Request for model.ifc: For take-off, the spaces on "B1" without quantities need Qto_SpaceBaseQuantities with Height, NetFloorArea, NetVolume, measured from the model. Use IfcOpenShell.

First a look at what the model holds.

```python
import ifcopenshell
import ifcopenshell.util.element
import ifcopenshell.util.unit

model = ifcopenshell.open("model.ifc")
print(model.schema)
for unit_type in ("LENGTHUNIT", "AREAUNIT", "VOLUMEUNIT"):
    print(unit_type, ifcopenshell.util.unit.calculate_unit_scale(model, unit_type))
storey = next(s for s in model.by_type("IfcBuildingStorey") if s.Name == "B1")
spaces = [e for e in ifcopenshell.util.element.get_decomposition(storey) if e.is_a("IfcSpace")]
for e in sorted(spaces, key=lambda e: e.id()):
    print(e.id(), e.is_a(), e.Name, list(ifcopenshell.util.element.get_psets(e, qtos_only=True)), sep=" | ")
```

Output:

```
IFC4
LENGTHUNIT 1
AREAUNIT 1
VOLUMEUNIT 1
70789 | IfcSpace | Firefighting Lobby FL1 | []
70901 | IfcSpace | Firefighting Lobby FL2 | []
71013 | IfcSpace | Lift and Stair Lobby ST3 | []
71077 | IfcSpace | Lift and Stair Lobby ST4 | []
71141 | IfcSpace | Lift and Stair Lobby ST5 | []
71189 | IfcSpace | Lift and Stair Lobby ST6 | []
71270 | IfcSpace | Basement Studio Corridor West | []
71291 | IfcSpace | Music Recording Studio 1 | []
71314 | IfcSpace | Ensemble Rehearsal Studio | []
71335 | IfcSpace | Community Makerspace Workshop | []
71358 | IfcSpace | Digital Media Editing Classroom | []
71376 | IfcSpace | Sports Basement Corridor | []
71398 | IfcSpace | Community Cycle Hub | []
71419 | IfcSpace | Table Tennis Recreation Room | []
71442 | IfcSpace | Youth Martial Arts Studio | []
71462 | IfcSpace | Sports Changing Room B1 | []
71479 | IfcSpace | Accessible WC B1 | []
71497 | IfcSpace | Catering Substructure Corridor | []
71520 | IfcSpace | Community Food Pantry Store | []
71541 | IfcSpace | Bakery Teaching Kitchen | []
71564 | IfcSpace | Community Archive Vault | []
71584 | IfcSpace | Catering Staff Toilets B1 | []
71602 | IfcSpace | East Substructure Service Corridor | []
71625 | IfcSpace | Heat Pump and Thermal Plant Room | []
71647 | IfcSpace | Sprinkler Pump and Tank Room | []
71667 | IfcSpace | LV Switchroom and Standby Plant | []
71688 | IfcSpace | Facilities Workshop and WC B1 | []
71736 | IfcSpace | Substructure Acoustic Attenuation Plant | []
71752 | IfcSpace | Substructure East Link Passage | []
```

```python
import ifcopenshell
import ifcopenshell.api.pset
import ifcopenshell.geom
import ifcopenshell.util.element
import ifcopenshell.util.shape
import ifcopenshell.util.unit

model = ifcopenshell.open("model.ifc")
unit_scale = ifcopenshell.util.unit.calculate_unit_scale(model)
area_scale = ifcopenshell.util.unit.calculate_unit_scale(model, "AREAUNIT")
volume_scale = ifcopenshell.util.unit.calculate_unit_scale(model, "VOLUMEUNIT")
settings = ifcopenshell.geom.settings()

storey = next(s for s in model.by_type("IfcBuildingStorey") if s.Name == "B1")
spaces = [e for e in ifcopenshell.util.element.get_decomposition(storey) if e.is_a("IfcSpace")]

for e in sorted(spaces, key=lambda e: e.id()):
    if ifcopenshell.util.element.get_psets(e, qtos_only=True, should_inherit=False):
        continue
    # Geometry comes back in metres, in the element's own axes.
    shape = ifcopenshell.geom.create_shape(settings, e)
    values = {
        "Height": ifcopenshell.util.shape.get_z(shape.geometry) / unit_scale,
        "NetFloorArea": ifcopenshell.util.shape.get_footprint_area(shape.geometry) / area_scale,
        "NetVolume": ifcopenshell.util.shape.get_volume(shape.geometry) / volume_scale,
    }
    qto = ifcopenshell.api.pset.add_qto(model, product=e, name="Qto_SpaceBaseQuantities")
    ifcopenshell.api.pset.edit_qto(model, qto=qto, properties=values)
    print(e.id(), {k: round(v, 3) for k, v in values.items()})

model.write("model_updated.ifc")
```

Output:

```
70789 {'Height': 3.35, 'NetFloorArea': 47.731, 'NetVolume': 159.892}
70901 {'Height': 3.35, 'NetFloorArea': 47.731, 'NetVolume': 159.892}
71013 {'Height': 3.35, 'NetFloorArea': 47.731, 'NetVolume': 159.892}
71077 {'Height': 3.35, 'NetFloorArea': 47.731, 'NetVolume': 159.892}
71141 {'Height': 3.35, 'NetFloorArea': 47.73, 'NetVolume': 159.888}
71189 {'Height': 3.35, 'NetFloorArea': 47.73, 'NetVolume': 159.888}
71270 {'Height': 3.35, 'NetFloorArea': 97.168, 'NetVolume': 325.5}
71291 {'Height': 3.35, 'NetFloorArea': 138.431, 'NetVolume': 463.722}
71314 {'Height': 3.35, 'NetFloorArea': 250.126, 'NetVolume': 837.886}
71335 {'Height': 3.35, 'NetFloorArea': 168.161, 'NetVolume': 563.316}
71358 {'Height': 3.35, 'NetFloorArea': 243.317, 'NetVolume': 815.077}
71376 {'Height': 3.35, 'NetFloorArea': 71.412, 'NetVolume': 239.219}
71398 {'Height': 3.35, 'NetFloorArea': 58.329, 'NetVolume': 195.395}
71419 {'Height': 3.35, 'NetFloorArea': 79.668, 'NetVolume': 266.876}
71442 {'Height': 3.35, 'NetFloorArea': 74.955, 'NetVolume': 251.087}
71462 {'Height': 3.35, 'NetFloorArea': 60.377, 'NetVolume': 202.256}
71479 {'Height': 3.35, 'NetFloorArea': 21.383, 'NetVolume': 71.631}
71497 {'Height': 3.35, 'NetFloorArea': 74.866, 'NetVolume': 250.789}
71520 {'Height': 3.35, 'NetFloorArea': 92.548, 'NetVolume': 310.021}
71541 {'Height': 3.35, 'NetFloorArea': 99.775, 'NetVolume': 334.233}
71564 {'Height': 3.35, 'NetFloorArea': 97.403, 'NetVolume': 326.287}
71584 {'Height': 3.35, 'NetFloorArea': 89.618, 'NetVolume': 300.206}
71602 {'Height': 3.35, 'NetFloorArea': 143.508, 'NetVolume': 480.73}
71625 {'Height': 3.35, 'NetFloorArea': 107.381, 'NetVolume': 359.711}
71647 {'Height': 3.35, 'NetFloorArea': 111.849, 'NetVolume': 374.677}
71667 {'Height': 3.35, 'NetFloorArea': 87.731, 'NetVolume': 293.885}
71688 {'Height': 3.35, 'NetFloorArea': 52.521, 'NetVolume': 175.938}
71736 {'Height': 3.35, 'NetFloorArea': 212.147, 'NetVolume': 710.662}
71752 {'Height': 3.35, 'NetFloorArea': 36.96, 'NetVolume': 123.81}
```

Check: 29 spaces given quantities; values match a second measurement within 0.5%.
